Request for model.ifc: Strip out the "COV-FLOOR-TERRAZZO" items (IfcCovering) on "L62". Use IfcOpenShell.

First a look at what the model holds.

```python
import ifcopenshell
import ifcopenshell.util.element

model = ifcopenshell.open("model.ifc")
print(model.schema)
storey = next(s for s in model.by_type("IfcBuildingStorey") if s.Name == "L62")
coverings = [e for e in ifcopenshell.util.element.get_decomposition(storey) if e.is_a("IfcCovering")]
seen = {}
for e in coverings:
    element_type = ifcopenshell.util.element.get_type(e)
    name = element_type.Name if element_type not in (None, e) else None
    seen[name] = seen.get(name, 0) + 1
for name, count in sorted(seen.items(), key=str):
    print(count, "x", name)
```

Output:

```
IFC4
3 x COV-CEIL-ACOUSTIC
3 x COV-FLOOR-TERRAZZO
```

```python
import ifcopenshell
import ifcopenshell.api.root
import ifcopenshell.util.element

model = ifcopenshell.open("model.ifc")

storey = next(s for s in model.by_type("IfcBuildingStorey") if s.Name == "L62")
coverings = [e for e in ifcopenshell.util.element.get_decomposition(storey) if e.is_a("IfcCovering")]
targets = [e for e in coverings if (t := ifcopenshell.util.element.get_type(e)) not in (None, e) and t.Name == "COV-FLOOR-TERRAZZO"]

for e in targets:
    ifcopenshell.api.root.remove_product(model, product=e)
print(len(targets), "removed")

model.write("model_edited.ifc")
```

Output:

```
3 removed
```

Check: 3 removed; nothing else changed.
